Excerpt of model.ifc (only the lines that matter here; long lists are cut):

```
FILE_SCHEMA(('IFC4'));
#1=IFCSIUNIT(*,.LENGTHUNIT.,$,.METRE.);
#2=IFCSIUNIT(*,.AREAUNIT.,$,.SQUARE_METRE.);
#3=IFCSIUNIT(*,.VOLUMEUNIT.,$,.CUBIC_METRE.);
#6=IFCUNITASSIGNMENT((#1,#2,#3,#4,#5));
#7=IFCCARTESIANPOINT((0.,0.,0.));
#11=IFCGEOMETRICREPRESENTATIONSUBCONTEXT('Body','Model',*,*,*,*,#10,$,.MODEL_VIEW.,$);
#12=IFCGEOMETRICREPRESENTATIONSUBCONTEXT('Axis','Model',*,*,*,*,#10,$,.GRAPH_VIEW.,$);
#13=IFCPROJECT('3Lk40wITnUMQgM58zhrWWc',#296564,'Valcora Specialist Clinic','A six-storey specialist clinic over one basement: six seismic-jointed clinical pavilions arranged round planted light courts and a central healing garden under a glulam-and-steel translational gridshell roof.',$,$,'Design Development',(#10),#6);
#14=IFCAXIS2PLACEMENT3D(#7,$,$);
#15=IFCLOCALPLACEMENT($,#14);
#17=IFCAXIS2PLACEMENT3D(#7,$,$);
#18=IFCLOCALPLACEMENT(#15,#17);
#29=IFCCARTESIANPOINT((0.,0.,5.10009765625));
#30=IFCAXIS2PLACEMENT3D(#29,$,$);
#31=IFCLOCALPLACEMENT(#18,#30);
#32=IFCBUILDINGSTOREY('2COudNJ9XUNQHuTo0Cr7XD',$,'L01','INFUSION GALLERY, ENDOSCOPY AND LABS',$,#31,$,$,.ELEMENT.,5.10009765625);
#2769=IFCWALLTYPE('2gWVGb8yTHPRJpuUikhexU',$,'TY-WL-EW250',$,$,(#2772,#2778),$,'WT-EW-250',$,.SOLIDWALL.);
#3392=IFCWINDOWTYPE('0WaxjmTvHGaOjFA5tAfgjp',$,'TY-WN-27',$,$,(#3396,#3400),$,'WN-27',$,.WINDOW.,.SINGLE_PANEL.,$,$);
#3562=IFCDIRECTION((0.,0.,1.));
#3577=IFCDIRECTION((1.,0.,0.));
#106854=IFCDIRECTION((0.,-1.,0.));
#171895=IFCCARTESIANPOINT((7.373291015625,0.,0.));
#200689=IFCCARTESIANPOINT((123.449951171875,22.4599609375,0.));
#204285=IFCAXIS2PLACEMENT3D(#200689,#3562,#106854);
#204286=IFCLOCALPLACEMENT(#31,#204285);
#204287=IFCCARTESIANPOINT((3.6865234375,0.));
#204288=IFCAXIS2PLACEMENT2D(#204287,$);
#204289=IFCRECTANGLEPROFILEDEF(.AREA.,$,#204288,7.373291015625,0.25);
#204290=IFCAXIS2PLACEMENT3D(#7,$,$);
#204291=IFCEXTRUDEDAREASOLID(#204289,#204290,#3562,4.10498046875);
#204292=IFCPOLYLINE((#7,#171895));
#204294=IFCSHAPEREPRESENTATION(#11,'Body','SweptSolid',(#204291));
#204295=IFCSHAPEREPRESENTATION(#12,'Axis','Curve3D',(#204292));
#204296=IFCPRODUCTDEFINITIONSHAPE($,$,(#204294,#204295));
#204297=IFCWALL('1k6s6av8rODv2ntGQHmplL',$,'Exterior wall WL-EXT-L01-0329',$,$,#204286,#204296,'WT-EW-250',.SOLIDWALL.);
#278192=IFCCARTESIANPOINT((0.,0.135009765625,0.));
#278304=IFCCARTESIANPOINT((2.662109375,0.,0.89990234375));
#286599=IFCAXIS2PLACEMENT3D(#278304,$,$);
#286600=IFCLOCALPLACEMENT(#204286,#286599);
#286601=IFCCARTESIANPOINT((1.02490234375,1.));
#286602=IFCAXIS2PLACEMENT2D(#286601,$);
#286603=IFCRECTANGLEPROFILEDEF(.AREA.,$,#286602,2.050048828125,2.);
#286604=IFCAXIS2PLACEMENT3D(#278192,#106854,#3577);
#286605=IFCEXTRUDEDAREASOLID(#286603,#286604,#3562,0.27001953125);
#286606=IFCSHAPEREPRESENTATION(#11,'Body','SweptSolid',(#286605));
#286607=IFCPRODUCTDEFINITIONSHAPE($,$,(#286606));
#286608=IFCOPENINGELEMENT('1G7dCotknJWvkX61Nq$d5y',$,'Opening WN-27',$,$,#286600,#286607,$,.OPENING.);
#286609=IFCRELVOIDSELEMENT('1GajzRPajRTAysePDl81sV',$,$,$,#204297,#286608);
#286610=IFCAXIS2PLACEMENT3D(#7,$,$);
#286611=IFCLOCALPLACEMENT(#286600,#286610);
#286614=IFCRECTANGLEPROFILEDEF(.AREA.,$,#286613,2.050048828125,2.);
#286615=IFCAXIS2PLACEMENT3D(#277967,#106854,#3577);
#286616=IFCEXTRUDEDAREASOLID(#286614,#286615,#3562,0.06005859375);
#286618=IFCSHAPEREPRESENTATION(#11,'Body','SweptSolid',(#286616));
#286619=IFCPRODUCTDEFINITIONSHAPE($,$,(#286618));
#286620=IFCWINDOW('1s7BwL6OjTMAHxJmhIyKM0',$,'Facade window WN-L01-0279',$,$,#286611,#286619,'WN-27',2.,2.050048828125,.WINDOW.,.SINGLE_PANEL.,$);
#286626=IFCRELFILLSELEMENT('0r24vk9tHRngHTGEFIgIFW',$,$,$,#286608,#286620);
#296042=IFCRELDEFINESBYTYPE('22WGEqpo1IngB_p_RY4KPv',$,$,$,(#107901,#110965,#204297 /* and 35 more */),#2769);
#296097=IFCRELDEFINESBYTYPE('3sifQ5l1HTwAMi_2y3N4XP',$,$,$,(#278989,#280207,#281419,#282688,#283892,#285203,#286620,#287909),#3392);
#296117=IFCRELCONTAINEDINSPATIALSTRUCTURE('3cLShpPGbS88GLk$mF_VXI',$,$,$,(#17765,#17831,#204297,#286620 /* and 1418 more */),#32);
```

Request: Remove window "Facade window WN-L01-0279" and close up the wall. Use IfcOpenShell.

```python
import ifcopenshell
import ifcopenshell.api.feature
import ifcopenshell.api.root
import ifcopenshell.geom
import ifcopenshell.util.shape

model = ifcopenshell.open("model.ifc")
settings = ifcopenshell.geom.settings()


def volume(element):
    """Net volume in cubic metres, openings subtracted."""
    shape = ifcopenshell.geom.create_shape(settings, element)
    return ifcopenshell.util.shape.get_volume(shape.geometry)


window = model.by_guid("1s7BwL6OjTMAHxJmhIyKM0")
opening = window.FillsVoids[0].RelatingOpeningElement
wall = opening.VoidsElements[0].RelatingBuildingElement
before = volume(wall)

ifcopenshell.api.root.remove_product(model, product=window)
ifcopenshell.api.feature.remove_feature(model, feature=opening)

after = volume(wall)

print(f"wall volume {before:.3f} -> {after:.3f} m3")

model.write("model_v2.ifc")
```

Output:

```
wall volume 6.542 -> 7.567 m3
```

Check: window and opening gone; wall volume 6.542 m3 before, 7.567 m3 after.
